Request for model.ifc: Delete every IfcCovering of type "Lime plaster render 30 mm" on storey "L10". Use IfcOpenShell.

First a look at what the model holds.

```python
import ifcopenshell
import ifcopenshell.util.element

model = ifcopenshell.open("model.ifc")
print(model.schema)
storey = next(s for s in model.by_type("IfcBuildingStorey") if s.Name == "L10")
coverings = [e for e in ifcopenshell.util.element.get_decomposition(storey) if e.is_a("IfcCovering")]
seen = {}
for e in coverings:
    element_type = ifcopenshell.util.element.get_type(e)
    name = element_type.Name if element_type not in (None, e) else None
    seen[name] = seen.get(name, 0) + 1
for name, count in sorted(seen.items(), key=str):
    print(count, "x", name)
```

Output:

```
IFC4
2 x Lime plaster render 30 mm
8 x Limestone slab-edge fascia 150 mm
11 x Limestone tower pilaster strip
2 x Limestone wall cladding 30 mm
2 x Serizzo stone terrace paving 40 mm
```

```python
import ifcopenshell
import ifcopenshell.api.root
import ifcopenshell.util.element

model = ifcopenshell.open("model.ifc")

storey = next(s for s in model.by_type("IfcBuildingStorey") if s.Name == "L10")
coverings = [e for e in ifcopenshell.util.element.get_decomposition(storey) if e.is_a("IfcCovering")]
targets = [e for e in coverings if (t := ifcopenshell.util.element.get_type(e)) not in (None, e) and t.Name == "Lime plaster render 30 mm"]

for e in targets:
    ifcopenshell.api.root.remove_product(model, product=e)
print(len(targets), "removed")

model.write("model_updated.ifc")
```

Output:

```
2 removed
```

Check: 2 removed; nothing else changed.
